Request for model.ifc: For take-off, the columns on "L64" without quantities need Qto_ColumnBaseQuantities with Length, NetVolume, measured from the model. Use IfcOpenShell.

First a look at what the model holds.

```python
import ifcopenshell
import ifcopenshell.util.element
import ifcopenshell.util.unit

model = ifcopenshell.open("model.ifc")
print(model.schema)
for unit_type in ("LENGTHUNIT", "AREAUNIT", "VOLUMEUNIT"):
    print(unit_type, ifcopenshell.util.unit.calculate_unit_scale(model, unit_type))
storey = next(s for s in model.by_type("IfcBuildingStorey") if s.Name == "L64")
columns = [e for e in ifcopenshell.util.element.get_decomposition(storey) if e.is_a("IfcColumn")]
for e in sorted(columns, key=lambda e: e.id()):
    print(e.id(), e.is_a(), e.Name, list(ifcopenshell.util.element.get_psets(e, qtos_only=True)), sep=" | ")
```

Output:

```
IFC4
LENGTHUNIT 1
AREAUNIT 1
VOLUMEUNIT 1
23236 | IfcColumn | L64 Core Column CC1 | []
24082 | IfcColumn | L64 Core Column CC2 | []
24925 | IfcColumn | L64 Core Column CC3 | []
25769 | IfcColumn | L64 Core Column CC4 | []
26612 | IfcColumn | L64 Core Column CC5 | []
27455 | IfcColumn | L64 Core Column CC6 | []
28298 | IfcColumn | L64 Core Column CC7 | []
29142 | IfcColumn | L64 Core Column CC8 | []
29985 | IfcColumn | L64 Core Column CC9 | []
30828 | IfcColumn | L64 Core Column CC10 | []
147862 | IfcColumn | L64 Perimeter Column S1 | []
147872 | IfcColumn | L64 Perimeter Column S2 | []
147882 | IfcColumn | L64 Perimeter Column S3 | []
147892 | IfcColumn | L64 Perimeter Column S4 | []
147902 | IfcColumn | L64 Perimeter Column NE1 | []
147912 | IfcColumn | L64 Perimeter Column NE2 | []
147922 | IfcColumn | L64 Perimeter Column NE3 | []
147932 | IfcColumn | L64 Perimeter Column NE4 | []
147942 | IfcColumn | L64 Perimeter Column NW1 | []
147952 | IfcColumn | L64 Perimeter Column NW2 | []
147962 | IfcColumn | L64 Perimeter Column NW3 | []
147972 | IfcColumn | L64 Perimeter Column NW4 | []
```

```python
import ifcopenshell
import ifcopenshell.api.pset
import ifcopenshell.geom
import ifcopenshell.util.element
import ifcopenshell.util.shape
import ifcopenshell.util.unit

model = ifcopenshell.open("model.ifc")
unit_scale = ifcopenshell.util.unit.calculate_unit_scale(model)
volume_scale = ifcopenshell.util.unit.calculate_unit_scale(model, "VOLUMEUNIT")
settings = ifcopenshell.geom.settings()

storey = next(s for s in model.by_type("IfcBuildingStorey") if s.Name == "L64")
columns = [e for e in ifcopenshell.util.element.get_decomposition(storey) if e.is_a("IfcColumn")]

for e in sorted(columns, key=lambda e: e.id()):
    if ifcopenshell.util.element.get_psets(e, qtos_only=True, should_inherit=False):
        continue
    # Geometry comes back in metres, in the element's own axes.
    shape = ifcopenshell.geom.create_shape(settings, e)
    values = {
        "Length": ifcopenshell.util.shape.get_z(shape.geometry) / unit_scale,
        "NetVolume": ifcopenshell.util.shape.get_volume(shape.geometry) / volume_scale,
    }
    qto = ifcopenshell.api.pset.add_qto(model, product=e, name="Qto_ColumnBaseQuantities")
    ifcopenshell.api.pset.edit_qto(model, qto=qto, properties=values)
    print(e.id(), {k: round(v, 3) for k, v in values.items()})

model.write("model-out.ifc")
```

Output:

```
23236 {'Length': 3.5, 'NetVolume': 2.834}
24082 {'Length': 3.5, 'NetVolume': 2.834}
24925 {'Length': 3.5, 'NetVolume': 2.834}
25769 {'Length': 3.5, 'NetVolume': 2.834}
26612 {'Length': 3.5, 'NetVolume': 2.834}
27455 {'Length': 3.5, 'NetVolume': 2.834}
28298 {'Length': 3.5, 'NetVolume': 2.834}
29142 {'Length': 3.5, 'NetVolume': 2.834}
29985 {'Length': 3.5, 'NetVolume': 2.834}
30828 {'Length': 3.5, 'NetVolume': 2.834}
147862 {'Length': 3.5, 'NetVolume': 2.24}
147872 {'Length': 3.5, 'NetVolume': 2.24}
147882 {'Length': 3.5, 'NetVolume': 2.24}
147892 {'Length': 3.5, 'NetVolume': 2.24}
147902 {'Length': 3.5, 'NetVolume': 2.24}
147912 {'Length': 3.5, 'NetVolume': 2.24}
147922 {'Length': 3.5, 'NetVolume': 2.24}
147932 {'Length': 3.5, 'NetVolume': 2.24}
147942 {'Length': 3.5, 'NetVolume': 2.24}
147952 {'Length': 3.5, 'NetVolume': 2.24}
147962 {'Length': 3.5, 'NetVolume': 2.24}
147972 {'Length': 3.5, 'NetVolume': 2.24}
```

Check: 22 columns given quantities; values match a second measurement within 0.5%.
